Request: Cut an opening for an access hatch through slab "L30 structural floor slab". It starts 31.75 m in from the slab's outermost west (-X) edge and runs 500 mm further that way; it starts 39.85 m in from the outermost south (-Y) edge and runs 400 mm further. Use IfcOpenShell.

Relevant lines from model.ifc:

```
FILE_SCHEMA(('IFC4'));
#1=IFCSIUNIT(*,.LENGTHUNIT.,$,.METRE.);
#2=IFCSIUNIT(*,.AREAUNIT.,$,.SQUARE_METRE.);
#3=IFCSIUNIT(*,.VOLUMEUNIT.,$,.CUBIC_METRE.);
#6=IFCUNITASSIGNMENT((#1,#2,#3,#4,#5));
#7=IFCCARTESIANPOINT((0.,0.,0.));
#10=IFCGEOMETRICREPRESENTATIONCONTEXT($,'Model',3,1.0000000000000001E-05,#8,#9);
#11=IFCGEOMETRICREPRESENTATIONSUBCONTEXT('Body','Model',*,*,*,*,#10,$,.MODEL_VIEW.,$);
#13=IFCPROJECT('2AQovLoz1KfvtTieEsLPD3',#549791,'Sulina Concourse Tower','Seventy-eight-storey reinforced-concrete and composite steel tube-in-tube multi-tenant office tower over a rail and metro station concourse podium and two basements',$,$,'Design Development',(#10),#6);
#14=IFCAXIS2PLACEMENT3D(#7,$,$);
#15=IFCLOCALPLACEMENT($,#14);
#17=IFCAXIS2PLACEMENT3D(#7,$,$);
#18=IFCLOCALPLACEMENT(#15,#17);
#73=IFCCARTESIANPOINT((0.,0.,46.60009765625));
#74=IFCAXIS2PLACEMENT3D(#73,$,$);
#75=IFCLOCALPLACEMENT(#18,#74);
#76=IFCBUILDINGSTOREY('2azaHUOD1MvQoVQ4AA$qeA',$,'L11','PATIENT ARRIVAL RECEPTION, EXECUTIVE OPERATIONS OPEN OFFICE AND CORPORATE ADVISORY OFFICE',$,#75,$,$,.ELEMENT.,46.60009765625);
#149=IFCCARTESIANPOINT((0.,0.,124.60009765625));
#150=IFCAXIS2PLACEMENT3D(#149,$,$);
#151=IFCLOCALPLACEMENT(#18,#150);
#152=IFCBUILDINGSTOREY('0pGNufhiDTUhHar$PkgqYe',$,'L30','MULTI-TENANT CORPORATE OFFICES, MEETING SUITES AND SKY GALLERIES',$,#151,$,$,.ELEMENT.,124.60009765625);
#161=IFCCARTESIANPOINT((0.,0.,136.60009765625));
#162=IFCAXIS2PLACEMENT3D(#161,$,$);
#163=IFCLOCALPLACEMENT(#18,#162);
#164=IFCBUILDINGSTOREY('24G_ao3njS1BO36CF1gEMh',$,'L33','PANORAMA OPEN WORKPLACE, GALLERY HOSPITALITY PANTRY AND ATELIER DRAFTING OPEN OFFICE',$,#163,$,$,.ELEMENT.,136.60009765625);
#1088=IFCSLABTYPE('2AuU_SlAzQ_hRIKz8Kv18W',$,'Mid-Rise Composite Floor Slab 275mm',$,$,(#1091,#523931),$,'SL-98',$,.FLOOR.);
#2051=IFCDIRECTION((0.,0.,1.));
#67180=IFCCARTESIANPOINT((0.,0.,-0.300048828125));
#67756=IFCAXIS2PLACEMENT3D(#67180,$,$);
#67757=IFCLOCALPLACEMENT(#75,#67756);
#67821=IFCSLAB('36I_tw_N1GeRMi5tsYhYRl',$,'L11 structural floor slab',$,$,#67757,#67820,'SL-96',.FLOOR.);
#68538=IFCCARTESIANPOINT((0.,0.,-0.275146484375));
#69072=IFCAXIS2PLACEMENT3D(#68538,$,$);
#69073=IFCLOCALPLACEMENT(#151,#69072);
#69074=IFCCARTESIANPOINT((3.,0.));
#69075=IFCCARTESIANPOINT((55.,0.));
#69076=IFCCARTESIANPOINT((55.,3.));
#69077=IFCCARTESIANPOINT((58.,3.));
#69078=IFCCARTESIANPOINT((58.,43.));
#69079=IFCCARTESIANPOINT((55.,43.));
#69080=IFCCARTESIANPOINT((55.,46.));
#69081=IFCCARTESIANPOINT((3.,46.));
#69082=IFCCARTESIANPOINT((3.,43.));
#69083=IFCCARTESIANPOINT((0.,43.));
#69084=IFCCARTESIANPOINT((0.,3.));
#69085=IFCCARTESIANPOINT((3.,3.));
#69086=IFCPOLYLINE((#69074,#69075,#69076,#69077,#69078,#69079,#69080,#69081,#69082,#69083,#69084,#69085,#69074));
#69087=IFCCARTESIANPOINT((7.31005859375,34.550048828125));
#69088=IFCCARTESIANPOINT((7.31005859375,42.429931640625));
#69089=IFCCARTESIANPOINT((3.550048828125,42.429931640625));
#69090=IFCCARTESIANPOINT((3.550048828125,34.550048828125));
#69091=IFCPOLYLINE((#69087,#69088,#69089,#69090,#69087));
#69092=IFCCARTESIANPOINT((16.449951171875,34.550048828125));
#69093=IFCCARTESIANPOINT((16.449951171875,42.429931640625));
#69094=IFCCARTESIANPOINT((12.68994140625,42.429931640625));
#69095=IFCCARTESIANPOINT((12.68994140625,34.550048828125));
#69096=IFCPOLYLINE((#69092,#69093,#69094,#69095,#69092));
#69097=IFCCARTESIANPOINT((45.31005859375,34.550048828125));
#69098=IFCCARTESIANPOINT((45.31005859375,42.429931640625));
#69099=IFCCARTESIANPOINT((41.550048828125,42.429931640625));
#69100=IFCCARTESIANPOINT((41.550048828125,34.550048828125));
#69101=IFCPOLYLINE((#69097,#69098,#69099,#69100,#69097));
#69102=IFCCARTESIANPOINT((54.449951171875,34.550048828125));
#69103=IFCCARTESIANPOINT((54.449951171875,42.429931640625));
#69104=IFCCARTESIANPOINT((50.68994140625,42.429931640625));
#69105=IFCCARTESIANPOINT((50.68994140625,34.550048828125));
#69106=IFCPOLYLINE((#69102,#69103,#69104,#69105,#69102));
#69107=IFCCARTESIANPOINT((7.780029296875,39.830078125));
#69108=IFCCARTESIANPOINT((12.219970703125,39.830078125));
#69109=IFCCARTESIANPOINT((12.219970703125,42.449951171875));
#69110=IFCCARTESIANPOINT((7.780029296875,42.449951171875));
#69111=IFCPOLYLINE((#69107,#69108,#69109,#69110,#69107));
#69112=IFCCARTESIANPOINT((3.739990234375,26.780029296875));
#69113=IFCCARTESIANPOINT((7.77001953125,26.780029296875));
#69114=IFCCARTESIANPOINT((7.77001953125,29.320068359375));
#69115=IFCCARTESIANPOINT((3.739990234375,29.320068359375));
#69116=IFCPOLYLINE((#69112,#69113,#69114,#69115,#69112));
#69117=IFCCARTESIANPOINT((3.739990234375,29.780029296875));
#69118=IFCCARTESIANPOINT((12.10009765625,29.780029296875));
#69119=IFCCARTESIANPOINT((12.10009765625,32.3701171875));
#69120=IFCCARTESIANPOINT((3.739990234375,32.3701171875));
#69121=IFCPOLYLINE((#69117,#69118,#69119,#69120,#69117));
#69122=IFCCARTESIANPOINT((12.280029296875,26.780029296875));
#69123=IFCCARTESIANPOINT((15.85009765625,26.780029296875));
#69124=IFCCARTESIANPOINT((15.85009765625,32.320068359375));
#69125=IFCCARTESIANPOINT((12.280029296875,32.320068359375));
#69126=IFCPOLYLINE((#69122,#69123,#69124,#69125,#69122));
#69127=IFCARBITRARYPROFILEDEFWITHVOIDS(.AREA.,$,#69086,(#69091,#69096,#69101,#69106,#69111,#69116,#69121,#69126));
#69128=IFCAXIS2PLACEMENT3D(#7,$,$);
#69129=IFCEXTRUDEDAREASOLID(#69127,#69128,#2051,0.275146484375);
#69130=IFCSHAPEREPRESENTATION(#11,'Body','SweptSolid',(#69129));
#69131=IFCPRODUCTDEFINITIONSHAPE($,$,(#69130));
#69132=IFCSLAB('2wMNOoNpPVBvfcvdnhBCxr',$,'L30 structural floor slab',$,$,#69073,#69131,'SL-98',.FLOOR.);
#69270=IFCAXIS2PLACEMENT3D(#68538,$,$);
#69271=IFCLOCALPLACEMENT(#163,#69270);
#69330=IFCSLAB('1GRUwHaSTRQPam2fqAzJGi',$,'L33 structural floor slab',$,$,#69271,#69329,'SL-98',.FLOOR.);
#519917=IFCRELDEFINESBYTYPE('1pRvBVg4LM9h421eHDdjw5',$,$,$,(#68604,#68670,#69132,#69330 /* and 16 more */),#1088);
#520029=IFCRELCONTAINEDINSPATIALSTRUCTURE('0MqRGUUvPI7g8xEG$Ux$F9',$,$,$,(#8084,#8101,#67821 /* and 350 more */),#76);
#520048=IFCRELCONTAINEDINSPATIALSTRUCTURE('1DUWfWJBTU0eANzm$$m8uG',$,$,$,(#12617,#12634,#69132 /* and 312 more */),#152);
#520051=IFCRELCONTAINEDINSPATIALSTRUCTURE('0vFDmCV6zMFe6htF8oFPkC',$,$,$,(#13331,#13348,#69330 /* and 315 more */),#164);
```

```python
import numpy as np
import ifcopenshell
import ifcopenshell.api.feature
import ifcopenshell.api.geometry
import ifcopenshell.api.root
import ifcopenshell.geom
import ifcopenshell.util.placement
import ifcopenshell.util.representation
import ifcopenshell.util.shape
import ifcopenshell.util.unit

model = ifcopenshell.open("model.ifc")
unit_scale = ifcopenshell.util.unit.calculate_unit_scale(model)
settings = ifcopenshell.geom.settings()


def volume(element):
    """Net volume in cubic metres, openings subtracted."""
    shape = ifcopenshell.geom.create_shape(settings, element)
    return ifcopenshell.util.shape.get_volume(shape.geometry)


slab = model.by_id(69132)
before = volume(slab)

# Extent in the slab's own axes, in metres. The edges named are its -X and -Y sides.
slab_shape = ifcopenshell.geom.create_shape(settings, slab)
vertices = ifcopenshell.util.shape.get_vertices(slab_shape.geometry)
x_min, y_min, bottom = vertices.min(axis=0)
top = vertices[:, 2].max()

opening = ifcopenshell.api.root.create_entity(model, ifc_class="IfcOpeningElement", name="Access hatch opening", predefined_type="OPENING")
context = ifcopenshell.util.representation.get_context(model, "Model", "Body", "MODEL_VIEW")
width, depth = 0.5, 0.4
outline = [(0.0, 0.0), (width, 0.0), (width, depth), (0.0, depth), (0.0, 0.0)]
# Overshoot both faces by 50 mm so the cut is clean.
shape = ifcopenshell.api.geometry.add_slab_representation(
    model, context=context, depth=top - bottom + 0.1, polyline=outline
)
ifcopenshell.api.geometry.assign_representation(model, product=opening, representation=shape)

matrix = ifcopenshell.util.placement.get_local_placement(slab.ObjectPlacement)
matrix[:, 3] = matrix @ np.append(np.array([x_min + 31.75, y_min + 39.85, bottom - 0.05]) / unit_scale, 1.0)
ifcopenshell.api.geometry.edit_object_placement(model, product=opening, matrix=matrix, is_si=False)
ifcopenshell.api.feature.add_feature(model, feature=opening, element=slab)

after = volume(slab)

print(f"slab volume {before:.3f} -> {after:.3f} m3")

model.write("model-out.ifc")
```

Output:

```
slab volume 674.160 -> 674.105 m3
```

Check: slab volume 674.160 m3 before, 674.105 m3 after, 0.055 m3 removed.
